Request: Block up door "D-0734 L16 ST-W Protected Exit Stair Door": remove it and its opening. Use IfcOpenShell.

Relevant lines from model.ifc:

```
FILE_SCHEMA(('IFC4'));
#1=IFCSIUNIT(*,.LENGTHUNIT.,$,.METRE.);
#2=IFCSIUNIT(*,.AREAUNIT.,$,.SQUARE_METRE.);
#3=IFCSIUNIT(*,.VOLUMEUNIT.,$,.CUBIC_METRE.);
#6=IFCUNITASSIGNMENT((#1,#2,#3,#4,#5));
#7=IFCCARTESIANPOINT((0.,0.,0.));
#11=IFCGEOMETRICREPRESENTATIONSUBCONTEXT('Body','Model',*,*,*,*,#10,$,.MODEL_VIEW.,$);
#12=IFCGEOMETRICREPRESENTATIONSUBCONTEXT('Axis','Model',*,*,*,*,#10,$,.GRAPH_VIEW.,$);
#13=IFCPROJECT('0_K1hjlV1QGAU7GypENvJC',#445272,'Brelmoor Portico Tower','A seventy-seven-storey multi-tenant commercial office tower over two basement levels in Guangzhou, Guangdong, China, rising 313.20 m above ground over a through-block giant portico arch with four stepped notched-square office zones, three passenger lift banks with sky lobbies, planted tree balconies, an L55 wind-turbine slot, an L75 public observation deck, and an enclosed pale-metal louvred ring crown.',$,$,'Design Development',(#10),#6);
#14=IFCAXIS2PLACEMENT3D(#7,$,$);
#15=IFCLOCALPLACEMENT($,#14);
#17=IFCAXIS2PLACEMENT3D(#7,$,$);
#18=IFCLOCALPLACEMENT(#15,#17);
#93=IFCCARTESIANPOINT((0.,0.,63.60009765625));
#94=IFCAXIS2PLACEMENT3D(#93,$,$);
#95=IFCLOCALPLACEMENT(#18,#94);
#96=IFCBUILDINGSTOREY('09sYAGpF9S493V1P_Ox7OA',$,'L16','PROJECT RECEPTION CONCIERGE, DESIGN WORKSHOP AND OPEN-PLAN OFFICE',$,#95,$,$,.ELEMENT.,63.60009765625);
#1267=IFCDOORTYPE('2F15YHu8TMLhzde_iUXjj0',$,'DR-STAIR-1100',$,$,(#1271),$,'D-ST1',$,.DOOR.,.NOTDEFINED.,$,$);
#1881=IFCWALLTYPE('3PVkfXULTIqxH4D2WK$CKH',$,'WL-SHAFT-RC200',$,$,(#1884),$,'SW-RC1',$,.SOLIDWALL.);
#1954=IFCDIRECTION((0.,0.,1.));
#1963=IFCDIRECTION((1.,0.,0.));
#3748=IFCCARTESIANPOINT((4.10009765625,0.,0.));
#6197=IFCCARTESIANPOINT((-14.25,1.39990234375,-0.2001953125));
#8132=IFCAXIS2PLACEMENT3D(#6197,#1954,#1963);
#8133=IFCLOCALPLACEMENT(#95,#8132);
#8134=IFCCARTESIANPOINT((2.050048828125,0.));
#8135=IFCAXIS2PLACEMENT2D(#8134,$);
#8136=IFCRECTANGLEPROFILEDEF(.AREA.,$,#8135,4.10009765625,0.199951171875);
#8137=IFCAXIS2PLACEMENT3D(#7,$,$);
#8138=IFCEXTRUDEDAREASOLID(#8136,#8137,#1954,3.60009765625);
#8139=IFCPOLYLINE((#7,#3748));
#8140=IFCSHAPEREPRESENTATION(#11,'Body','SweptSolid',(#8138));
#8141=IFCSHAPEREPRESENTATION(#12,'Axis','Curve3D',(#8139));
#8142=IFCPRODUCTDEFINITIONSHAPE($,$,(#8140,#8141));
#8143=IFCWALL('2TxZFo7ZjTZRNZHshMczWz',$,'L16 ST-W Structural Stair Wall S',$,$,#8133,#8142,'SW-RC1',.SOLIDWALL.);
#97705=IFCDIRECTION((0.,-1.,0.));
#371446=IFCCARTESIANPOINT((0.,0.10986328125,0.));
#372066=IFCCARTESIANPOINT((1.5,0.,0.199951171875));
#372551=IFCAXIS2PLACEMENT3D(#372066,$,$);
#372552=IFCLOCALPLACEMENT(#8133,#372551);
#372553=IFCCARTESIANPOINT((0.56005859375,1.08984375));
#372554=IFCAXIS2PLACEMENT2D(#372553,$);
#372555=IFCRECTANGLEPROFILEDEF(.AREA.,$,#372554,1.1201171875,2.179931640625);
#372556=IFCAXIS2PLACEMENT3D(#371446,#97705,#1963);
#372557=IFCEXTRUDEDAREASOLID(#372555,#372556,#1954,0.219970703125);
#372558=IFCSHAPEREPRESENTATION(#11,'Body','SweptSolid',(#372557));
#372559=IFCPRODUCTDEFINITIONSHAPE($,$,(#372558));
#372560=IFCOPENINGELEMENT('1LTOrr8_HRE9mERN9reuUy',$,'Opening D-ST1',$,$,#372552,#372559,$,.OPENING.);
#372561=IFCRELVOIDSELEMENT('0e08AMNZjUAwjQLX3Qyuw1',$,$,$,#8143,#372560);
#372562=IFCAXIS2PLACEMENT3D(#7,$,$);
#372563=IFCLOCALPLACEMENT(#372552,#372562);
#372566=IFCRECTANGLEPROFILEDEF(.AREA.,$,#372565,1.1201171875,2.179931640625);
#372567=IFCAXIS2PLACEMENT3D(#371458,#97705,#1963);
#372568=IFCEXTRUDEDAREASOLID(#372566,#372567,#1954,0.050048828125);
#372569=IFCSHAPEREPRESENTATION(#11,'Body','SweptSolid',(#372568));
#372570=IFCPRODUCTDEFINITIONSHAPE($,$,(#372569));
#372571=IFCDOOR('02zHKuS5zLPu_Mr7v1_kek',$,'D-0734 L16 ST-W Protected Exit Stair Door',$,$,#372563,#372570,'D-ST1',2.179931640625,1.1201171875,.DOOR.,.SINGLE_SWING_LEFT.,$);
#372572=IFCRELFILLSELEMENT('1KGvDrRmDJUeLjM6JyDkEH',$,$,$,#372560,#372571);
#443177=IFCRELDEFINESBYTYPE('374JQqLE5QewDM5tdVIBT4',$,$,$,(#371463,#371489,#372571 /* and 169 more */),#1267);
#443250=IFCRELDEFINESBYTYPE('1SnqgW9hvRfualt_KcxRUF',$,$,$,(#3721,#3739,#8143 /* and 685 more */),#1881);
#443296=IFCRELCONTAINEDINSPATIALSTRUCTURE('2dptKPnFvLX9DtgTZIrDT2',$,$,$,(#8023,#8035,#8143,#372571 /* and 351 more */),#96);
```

```python
import ifcopenshell
import ifcopenshell.api.feature
import ifcopenshell.api.root
import ifcopenshell.geom
import ifcopenshell.util.shape

model = ifcopenshell.open("model.ifc")
settings = ifcopenshell.geom.settings()


def volume(element):
    """Net volume in cubic metres, openings subtracted."""
    shape = ifcopenshell.geom.create_shape(settings, element)
    return ifcopenshell.util.shape.get_volume(shape.geometry)


door = model.by_id(372571)
opening = door.FillsVoids[0].RelatingOpeningElement
wall = opening.VoidsElements[0].RelatingBuildingElement
before = volume(wall)

ifcopenshell.api.root.remove_product(model, product=door)
ifcopenshell.api.feature.remove_feature(model, feature=opening)

after = volume(wall)

print(f"wall volume {before:.3f} -> {after:.3f} m3")

model.write("model-out.ifc")
```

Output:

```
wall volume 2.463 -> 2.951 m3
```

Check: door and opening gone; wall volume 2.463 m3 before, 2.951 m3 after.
